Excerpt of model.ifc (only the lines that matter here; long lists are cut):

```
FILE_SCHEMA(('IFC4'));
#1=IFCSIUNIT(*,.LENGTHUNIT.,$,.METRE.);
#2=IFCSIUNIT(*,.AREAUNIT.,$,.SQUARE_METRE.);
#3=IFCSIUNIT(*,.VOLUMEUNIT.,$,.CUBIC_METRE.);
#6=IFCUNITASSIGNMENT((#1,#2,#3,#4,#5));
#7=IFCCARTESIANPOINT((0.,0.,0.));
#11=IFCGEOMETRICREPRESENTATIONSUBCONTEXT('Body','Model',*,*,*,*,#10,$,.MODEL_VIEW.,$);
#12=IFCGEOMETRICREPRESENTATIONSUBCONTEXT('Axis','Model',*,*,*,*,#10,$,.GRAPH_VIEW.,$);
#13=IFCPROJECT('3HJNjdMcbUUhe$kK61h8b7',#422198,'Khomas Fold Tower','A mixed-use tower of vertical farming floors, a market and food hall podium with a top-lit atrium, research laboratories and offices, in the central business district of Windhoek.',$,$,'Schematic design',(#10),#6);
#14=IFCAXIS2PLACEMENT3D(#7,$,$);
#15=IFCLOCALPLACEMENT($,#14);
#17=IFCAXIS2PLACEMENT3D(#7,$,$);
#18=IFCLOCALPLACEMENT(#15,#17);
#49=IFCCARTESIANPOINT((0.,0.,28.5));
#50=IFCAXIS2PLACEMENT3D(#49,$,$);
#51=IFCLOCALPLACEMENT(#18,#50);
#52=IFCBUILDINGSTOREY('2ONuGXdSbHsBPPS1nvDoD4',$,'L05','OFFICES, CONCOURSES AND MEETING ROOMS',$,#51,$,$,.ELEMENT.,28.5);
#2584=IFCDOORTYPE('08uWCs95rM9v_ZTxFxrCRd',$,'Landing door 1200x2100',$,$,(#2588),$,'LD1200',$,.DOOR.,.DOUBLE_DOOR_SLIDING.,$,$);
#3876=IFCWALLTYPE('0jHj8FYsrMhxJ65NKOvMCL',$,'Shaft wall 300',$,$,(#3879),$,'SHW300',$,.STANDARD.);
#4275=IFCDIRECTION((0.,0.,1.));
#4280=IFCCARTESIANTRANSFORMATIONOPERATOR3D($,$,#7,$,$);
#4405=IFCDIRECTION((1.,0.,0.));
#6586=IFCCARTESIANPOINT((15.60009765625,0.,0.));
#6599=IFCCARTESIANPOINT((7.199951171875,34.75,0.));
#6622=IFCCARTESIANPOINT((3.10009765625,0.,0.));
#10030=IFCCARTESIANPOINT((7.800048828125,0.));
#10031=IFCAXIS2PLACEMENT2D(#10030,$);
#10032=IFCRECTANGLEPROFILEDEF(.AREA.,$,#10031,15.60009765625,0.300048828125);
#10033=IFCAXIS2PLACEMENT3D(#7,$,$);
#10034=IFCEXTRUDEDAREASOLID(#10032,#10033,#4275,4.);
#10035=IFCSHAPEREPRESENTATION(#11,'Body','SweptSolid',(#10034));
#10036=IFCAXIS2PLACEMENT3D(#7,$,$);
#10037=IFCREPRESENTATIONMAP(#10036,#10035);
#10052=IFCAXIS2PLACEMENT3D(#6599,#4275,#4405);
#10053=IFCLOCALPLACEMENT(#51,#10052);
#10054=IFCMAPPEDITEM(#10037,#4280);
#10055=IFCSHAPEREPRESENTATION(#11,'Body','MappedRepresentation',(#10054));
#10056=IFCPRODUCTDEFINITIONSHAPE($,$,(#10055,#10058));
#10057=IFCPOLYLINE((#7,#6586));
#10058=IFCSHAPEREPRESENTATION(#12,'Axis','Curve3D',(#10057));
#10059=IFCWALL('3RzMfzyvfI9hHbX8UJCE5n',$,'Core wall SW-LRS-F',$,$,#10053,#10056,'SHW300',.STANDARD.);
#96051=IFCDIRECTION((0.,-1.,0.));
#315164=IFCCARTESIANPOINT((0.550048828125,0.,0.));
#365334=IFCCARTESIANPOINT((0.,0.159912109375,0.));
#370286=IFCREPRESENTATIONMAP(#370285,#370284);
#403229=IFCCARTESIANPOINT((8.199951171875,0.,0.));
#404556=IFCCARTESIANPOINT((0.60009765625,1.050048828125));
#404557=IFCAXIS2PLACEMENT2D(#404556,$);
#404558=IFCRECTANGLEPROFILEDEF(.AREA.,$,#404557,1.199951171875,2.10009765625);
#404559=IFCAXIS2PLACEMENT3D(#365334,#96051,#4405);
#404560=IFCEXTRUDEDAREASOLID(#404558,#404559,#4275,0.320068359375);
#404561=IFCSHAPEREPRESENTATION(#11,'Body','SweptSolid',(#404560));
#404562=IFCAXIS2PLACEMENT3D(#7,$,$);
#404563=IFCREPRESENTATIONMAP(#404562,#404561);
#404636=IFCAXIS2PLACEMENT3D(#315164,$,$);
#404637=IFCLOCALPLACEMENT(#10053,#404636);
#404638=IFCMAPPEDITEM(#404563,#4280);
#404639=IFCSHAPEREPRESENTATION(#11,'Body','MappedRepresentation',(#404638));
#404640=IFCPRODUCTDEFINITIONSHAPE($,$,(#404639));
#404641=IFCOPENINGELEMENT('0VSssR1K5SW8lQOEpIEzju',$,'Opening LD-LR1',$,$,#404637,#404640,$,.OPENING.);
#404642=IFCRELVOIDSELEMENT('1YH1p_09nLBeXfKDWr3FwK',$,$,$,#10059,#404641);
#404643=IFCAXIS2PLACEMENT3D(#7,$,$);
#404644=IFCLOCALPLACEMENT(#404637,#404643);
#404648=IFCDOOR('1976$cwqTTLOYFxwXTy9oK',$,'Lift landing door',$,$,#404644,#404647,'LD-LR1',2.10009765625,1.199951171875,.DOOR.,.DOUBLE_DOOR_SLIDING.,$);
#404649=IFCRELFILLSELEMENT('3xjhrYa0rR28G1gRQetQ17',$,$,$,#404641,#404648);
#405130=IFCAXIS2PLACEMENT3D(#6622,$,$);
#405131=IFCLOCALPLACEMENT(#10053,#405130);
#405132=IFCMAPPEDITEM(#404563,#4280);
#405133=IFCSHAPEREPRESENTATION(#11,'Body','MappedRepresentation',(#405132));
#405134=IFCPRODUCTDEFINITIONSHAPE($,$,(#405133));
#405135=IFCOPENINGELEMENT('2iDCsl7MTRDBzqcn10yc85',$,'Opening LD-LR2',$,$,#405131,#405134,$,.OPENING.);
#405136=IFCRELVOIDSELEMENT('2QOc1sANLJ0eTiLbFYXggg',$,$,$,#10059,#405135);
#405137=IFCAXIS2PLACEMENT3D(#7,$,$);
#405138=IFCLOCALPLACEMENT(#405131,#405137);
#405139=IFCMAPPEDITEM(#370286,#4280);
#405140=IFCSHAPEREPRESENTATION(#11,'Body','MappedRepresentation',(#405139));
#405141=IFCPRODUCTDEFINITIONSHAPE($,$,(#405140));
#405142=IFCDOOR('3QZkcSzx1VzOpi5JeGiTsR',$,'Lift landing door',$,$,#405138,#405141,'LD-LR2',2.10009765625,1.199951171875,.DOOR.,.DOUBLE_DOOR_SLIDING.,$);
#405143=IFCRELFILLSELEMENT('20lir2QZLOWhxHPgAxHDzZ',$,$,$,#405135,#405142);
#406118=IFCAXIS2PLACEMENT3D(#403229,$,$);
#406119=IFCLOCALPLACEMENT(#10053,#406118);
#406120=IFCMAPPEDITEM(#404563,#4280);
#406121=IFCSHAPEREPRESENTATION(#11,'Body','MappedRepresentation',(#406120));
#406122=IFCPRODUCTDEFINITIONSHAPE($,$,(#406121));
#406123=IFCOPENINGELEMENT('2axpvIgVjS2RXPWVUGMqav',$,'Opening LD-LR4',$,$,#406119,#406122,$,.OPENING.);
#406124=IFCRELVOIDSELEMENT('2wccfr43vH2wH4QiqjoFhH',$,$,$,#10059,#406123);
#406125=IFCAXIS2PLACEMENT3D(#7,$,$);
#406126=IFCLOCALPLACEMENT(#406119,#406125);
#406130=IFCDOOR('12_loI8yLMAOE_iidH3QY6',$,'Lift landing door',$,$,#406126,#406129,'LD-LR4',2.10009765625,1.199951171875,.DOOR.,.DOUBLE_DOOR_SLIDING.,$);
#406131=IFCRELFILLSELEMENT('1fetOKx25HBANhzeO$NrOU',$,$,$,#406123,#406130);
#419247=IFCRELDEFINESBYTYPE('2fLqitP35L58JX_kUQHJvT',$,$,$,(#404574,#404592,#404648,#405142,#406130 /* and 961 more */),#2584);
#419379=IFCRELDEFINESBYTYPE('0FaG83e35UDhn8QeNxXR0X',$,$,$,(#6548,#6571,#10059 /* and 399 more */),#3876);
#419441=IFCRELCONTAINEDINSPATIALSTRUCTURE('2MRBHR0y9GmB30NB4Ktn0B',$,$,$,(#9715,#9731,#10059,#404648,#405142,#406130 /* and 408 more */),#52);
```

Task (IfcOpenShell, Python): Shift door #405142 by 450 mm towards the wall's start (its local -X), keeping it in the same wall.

```python
import ifcopenshell
import ifcopenshell.api.geometry
import ifcopenshell.util.placement

model = ifcopenshell.open("model.ifc")

door = model.by_guid("3QZkcSzx1VzOpi5JeGiTsR")
opening = door.FillsVoids[0].RelatingOpeningElement
wall = opening.VoidsElements[0].RelatingBuildingElement

wall_matrix = ifcopenshell.util.placement.get_local_placement(wall.ObjectPlacement)
shift = wall_matrix[:3, 0] * -0.45
before = ifcopenshell.util.placement.get_local_placement(door.ObjectPlacement)[:3, 3].copy()

# The door is placed relative to its opening, so it follows when the opening moves.
matrix = ifcopenshell.util.placement.get_local_placement(opening.ObjectPlacement)
matrix[:3, 3] += shift
ifcopenshell.api.geometry.edit_object_placement(
    model, product=opening, matrix=matrix, is_si=False, should_transform_children=True
)

after = ifcopenshell.util.placement.get_local_placement(door.ObjectPlacement)[:3, 3]
print("door moved by", (after - before).round(3) + 0.0)

model.write("model_edited.ifc")
```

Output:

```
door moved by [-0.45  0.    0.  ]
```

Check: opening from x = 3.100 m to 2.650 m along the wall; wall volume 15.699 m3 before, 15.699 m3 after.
